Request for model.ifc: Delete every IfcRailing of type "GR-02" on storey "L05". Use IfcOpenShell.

First a look at what the model holds.

```python
import ifcopenshell
import ifcopenshell.util.element

model = ifcopenshell.open("model.ifc")
print(model.schema)
storey = next(s for s in model.by_type("IfcBuildingStorey") if s.Name == "L05")
railings = [e for e in ifcopenshell.util.element.get_decomposition(storey) if e.is_a("IfcRailing")]
seen = {}
for e in railings:
    element_type = ifcopenshell.util.element.get_type(e)
    name = element_type.Name if element_type not in (None, e) else None
    seen[name] = seen.get(name, 0) + 1
for name, count in sorted(seen.items(), key=str):
    print(count, "x", name)
```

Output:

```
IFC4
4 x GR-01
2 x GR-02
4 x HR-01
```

```python
import ifcopenshell
import ifcopenshell.api.root
import ifcopenshell.util.element

model = ifcopenshell.open("model.ifc")

storey = next(s for s in model.by_type("IfcBuildingStorey") if s.Name == "L05")
railings = [e for e in ifcopenshell.util.element.get_decomposition(storey) if e.is_a("IfcRailing")]
targets = [e for e in railings if (t := ifcopenshell.util.element.get_type(e)) not in (None, e) and t.Name == "GR-02"]

for e in targets:
    ifcopenshell.api.root.remove_product(model, product=e)
print(len(targets), "removed")

model.write("model-out.ifc")
```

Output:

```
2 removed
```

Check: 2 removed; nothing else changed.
